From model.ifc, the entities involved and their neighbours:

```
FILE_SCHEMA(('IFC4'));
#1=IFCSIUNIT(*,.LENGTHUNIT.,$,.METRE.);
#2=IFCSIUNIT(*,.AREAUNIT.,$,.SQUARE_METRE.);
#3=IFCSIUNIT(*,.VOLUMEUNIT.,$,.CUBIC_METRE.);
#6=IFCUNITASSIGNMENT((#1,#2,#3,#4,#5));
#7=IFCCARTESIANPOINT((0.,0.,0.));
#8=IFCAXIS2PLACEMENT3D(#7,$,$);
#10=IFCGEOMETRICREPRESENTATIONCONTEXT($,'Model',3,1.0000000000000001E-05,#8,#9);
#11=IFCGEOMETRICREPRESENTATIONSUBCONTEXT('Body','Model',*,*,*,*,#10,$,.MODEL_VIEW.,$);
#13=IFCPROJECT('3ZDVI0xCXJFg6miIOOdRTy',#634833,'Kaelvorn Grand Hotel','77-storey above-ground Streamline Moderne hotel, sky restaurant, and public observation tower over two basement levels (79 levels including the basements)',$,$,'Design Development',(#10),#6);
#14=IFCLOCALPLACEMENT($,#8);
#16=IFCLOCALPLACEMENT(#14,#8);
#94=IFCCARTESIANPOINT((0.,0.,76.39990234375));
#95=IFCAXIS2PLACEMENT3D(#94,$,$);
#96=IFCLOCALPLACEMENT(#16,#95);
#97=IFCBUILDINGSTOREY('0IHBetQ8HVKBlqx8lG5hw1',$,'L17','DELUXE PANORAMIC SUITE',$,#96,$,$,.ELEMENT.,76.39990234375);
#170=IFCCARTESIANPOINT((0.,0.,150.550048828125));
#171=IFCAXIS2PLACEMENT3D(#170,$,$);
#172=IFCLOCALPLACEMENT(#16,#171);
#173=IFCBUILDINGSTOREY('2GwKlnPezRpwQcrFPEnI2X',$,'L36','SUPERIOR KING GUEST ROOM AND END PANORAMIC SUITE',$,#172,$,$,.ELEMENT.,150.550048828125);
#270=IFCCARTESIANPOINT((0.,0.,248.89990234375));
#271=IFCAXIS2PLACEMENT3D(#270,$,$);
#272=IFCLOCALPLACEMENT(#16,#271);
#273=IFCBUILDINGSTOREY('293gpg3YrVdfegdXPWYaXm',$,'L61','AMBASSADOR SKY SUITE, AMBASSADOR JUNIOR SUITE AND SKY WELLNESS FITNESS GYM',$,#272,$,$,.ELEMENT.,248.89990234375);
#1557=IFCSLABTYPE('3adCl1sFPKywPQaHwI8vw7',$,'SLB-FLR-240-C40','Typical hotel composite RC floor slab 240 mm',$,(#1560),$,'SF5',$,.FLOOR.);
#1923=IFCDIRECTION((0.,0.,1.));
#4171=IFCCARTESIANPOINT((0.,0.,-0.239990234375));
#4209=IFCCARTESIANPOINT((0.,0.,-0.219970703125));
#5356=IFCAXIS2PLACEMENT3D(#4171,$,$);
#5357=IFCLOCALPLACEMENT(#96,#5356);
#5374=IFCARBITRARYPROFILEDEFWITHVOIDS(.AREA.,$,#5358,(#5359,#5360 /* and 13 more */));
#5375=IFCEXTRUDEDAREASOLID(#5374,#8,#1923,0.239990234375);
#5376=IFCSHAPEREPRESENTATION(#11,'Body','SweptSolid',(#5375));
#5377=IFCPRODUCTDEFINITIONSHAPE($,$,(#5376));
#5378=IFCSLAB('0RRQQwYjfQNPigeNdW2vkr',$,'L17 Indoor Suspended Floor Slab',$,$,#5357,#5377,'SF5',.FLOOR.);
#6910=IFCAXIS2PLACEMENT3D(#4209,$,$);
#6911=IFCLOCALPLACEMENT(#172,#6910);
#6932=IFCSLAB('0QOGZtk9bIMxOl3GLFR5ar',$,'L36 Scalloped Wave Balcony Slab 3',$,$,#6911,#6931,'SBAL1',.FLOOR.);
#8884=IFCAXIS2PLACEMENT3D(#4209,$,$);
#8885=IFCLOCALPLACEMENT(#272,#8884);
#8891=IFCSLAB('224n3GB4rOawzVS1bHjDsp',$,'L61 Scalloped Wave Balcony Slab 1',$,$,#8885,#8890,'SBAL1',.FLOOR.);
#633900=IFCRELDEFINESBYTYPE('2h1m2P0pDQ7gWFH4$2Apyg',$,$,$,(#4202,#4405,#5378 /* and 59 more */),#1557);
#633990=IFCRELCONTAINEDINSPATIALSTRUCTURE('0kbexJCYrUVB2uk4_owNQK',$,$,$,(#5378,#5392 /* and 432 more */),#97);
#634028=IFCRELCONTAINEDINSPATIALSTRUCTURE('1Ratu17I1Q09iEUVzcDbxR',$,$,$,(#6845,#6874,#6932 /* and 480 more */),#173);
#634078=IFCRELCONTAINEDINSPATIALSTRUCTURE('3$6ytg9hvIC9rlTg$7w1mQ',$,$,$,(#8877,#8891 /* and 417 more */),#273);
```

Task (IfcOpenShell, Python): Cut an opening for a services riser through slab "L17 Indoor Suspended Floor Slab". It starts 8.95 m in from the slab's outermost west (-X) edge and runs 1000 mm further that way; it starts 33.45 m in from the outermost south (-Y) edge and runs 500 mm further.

```python
import numpy as np
import ifcopenshell
import ifcopenshell.api.feature
import ifcopenshell.api.geometry
import ifcopenshell.api.root
import ifcopenshell.geom
import ifcopenshell.util.placement
import ifcopenshell.util.representation
import ifcopenshell.util.shape
import ifcopenshell.util.unit

model = ifcopenshell.open("model.ifc")
unit_scale = ifcopenshell.util.unit.calculate_unit_scale(model)
settings = ifcopenshell.geom.settings()


def volume(element):
    """Net volume in cubic metres, openings subtracted."""
    shape = ifcopenshell.geom.create_shape(settings, element)
    return ifcopenshell.util.shape.get_volume(shape.geometry)


slab = model.by_guid("0RRQQwYjfQNPigeNdW2vkr")
before = volume(slab)

# Extent in the slab's own axes, in metres. The edges named are its -X and -Y sides.
slab_shape = ifcopenshell.geom.create_shape(settings, slab)
vertices = ifcopenshell.util.shape.get_vertices(slab_shape.geometry)
x_min, y_min, bottom = vertices.min(axis=0)
top = vertices[:, 2].max()

opening = ifcopenshell.api.root.create_entity(model, ifc_class="IfcOpeningElement", name="Services riser opening", predefined_type="OPENING")
context = ifcopenshell.util.representation.get_context(model, "Model", "Body", "MODEL_VIEW")
width, depth = 1, 0.5
outline = [(0.0, 0.0), (width, 0.0), (width, depth), (0.0, depth), (0.0, 0.0)]
# Overshoot both faces by 50 mm so the cut is clean.
shape = ifcopenshell.api.geometry.add_slab_representation(
    model, context=context, depth=top - bottom + 0.1, polyline=outline
)
ifcopenshell.api.geometry.assign_representation(model, product=opening, representation=shape)

matrix = ifcopenshell.util.placement.get_local_placement(slab.ObjectPlacement)
matrix[:, 3] = matrix @ np.append(np.array([x_min + 8.95, y_min + 33.45, bottom - 0.05]) / unit_scale, 1.0)
ifcopenshell.api.geometry.edit_object_placement(model, product=opening, matrix=matrix, is_si=False)
ifcopenshell.api.feature.add_feature(model, feature=opening, element=slab)

after = volume(slab)

print(f"slab volume {before:.3f} -> {after:.3f} m3")

model.write("model_v2.ifc")
```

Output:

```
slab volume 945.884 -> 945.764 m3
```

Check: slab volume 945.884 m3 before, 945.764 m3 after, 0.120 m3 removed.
